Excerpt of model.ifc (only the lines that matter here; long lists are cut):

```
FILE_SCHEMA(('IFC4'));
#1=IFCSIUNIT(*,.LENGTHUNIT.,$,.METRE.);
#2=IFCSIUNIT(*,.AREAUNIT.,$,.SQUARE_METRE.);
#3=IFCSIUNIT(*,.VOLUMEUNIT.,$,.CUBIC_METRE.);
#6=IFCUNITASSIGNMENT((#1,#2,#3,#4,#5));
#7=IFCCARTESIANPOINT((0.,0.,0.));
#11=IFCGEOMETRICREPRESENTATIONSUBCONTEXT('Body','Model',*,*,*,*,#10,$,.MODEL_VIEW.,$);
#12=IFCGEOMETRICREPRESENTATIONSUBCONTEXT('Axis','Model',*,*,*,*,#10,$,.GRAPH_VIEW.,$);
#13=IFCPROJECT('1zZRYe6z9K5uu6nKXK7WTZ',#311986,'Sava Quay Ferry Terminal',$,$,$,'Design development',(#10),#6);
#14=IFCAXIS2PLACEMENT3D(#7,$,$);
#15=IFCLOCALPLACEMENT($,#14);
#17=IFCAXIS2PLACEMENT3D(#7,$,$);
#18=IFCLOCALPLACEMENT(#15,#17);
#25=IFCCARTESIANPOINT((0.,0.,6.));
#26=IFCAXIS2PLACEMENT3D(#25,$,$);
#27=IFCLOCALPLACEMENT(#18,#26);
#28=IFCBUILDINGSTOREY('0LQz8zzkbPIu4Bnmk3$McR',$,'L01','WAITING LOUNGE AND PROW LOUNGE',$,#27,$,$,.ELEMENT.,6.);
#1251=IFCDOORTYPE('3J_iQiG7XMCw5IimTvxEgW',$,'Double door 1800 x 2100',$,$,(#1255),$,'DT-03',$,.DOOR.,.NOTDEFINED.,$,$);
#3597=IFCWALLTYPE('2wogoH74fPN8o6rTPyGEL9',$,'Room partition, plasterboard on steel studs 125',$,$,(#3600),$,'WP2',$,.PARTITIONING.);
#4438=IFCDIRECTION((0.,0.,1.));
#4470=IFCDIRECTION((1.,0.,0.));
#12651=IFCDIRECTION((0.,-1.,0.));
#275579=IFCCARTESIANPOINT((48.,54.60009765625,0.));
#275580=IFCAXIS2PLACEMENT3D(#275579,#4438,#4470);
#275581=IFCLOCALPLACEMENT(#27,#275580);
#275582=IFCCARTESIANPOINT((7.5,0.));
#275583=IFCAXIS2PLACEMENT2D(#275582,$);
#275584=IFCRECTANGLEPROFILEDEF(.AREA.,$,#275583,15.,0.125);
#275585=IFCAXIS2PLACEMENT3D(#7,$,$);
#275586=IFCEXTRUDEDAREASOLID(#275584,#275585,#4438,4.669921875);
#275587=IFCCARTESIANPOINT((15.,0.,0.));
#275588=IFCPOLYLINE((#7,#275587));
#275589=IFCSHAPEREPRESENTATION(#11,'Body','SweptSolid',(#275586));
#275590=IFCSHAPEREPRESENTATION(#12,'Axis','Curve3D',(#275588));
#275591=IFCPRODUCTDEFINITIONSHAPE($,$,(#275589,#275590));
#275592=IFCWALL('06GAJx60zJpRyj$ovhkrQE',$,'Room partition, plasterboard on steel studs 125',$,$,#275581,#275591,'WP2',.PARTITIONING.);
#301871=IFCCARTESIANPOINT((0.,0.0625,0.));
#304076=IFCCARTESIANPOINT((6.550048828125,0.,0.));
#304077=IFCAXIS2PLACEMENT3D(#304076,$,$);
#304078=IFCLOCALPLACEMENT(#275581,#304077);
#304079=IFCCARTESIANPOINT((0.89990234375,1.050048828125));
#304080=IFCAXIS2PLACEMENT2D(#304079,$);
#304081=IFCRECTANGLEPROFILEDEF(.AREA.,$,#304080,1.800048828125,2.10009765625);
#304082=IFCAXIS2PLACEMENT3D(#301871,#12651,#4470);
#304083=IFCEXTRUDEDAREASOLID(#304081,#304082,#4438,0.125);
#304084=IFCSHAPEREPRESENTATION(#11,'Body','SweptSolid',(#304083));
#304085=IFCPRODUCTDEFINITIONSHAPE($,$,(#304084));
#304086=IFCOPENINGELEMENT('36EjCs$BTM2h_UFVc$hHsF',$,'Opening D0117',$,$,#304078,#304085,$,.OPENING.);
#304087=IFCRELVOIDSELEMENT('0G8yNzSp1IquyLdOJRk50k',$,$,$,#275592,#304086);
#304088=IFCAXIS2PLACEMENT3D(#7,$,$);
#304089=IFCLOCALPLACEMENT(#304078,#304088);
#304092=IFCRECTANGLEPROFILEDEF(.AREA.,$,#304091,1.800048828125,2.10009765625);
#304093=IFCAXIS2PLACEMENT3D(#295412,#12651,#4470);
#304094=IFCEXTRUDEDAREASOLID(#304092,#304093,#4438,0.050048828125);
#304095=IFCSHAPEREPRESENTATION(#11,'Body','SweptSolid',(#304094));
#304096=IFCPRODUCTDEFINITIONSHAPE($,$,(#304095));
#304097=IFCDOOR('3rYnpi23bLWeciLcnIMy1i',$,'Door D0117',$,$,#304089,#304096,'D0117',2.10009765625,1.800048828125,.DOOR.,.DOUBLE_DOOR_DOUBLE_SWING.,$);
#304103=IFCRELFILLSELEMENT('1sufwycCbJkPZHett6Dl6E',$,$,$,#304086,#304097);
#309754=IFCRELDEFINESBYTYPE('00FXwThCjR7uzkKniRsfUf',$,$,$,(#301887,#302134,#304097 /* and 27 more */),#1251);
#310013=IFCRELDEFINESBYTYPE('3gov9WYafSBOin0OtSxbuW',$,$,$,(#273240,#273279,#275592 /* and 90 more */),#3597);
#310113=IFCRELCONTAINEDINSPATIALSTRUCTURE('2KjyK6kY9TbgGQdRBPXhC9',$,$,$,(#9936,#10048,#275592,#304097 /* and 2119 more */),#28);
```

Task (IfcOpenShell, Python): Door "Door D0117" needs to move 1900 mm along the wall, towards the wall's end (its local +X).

```python
import ifcopenshell
import ifcopenshell.api.geometry
import ifcopenshell.util.placement
import ifcopenshell.util.unit

model = ifcopenshell.open("model.ifc")
unit_scale = ifcopenshell.util.unit.calculate_unit_scale(model)

door = model.by_guid("3rYnpi23bLWeciLcnIMy1i")
opening = door.FillsVoids[0].RelatingOpeningElement
wall = opening.VoidsElements[0].RelatingBuildingElement

wall_matrix = ifcopenshell.util.placement.get_local_placement(wall.ObjectPlacement)
shift = wall_matrix[:3, 0] * 1.9 / unit_scale
before = ifcopenshell.util.placement.get_local_placement(door.ObjectPlacement)[:3, 3].copy()

# The door is placed relative to its opening, so it follows when the opening moves.
matrix = ifcopenshell.util.placement.get_local_placement(opening.ObjectPlacement)
matrix[:3, 3] += shift
ifcopenshell.api.geometry.edit_object_placement(
    model, product=opening, matrix=matrix, is_si=False, should_transform_children=True
)

after = ifcopenshell.util.placement.get_local_placement(door.ObjectPlacement)[:3, 3]
print("door moved by", (after - before).round(3) + 0.0)

model.write("model_edited.ifc")
```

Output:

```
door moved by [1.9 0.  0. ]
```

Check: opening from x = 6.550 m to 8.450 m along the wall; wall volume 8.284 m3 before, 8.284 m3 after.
